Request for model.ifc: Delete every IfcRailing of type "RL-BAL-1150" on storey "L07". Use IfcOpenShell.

First a look at what the model holds.

```python
import ifcopenshell
import ifcopenshell.util.element

model = ifcopenshell.open("model.ifc")
print(model.schema)
storey = next(s for s in model.by_type("IfcBuildingStorey") if s.Name == "L07")
railings = [e for e in ifcopenshell.util.element.get_decomposition(storey) if e.is_a("IfcRailing")]
seen = {}
for e in railings:
    element_type = ifcopenshell.util.element.get_type(e)
    name = element_type.Name if element_type not in (None, e) else None
    seen[name] = seen.get(name, 0) + 1
for name, count in sorted(seen.items(), key=str):
    print(count, "x", name)
```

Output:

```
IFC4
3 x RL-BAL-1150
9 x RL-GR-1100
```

```python
import ifcopenshell
import ifcopenshell.api.root
import ifcopenshell.util.element

model = ifcopenshell.open("model.ifc")

storey = next(s for s in model.by_type("IfcBuildingStorey") if s.Name == "L07")
railings = [e for e in ifcopenshell.util.element.get_decomposition(storey) if e.is_a("IfcRailing")]
targets = [e for e in railings if (t := ifcopenshell.util.element.get_type(e)) not in (None, e) and t.Name == "RL-BAL-1150"]

for e in targets:
    ifcopenshell.api.root.remove_product(model, product=e)
print(len(targets), "removed")

model.write("model_updated.ifc")
```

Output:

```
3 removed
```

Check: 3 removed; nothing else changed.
